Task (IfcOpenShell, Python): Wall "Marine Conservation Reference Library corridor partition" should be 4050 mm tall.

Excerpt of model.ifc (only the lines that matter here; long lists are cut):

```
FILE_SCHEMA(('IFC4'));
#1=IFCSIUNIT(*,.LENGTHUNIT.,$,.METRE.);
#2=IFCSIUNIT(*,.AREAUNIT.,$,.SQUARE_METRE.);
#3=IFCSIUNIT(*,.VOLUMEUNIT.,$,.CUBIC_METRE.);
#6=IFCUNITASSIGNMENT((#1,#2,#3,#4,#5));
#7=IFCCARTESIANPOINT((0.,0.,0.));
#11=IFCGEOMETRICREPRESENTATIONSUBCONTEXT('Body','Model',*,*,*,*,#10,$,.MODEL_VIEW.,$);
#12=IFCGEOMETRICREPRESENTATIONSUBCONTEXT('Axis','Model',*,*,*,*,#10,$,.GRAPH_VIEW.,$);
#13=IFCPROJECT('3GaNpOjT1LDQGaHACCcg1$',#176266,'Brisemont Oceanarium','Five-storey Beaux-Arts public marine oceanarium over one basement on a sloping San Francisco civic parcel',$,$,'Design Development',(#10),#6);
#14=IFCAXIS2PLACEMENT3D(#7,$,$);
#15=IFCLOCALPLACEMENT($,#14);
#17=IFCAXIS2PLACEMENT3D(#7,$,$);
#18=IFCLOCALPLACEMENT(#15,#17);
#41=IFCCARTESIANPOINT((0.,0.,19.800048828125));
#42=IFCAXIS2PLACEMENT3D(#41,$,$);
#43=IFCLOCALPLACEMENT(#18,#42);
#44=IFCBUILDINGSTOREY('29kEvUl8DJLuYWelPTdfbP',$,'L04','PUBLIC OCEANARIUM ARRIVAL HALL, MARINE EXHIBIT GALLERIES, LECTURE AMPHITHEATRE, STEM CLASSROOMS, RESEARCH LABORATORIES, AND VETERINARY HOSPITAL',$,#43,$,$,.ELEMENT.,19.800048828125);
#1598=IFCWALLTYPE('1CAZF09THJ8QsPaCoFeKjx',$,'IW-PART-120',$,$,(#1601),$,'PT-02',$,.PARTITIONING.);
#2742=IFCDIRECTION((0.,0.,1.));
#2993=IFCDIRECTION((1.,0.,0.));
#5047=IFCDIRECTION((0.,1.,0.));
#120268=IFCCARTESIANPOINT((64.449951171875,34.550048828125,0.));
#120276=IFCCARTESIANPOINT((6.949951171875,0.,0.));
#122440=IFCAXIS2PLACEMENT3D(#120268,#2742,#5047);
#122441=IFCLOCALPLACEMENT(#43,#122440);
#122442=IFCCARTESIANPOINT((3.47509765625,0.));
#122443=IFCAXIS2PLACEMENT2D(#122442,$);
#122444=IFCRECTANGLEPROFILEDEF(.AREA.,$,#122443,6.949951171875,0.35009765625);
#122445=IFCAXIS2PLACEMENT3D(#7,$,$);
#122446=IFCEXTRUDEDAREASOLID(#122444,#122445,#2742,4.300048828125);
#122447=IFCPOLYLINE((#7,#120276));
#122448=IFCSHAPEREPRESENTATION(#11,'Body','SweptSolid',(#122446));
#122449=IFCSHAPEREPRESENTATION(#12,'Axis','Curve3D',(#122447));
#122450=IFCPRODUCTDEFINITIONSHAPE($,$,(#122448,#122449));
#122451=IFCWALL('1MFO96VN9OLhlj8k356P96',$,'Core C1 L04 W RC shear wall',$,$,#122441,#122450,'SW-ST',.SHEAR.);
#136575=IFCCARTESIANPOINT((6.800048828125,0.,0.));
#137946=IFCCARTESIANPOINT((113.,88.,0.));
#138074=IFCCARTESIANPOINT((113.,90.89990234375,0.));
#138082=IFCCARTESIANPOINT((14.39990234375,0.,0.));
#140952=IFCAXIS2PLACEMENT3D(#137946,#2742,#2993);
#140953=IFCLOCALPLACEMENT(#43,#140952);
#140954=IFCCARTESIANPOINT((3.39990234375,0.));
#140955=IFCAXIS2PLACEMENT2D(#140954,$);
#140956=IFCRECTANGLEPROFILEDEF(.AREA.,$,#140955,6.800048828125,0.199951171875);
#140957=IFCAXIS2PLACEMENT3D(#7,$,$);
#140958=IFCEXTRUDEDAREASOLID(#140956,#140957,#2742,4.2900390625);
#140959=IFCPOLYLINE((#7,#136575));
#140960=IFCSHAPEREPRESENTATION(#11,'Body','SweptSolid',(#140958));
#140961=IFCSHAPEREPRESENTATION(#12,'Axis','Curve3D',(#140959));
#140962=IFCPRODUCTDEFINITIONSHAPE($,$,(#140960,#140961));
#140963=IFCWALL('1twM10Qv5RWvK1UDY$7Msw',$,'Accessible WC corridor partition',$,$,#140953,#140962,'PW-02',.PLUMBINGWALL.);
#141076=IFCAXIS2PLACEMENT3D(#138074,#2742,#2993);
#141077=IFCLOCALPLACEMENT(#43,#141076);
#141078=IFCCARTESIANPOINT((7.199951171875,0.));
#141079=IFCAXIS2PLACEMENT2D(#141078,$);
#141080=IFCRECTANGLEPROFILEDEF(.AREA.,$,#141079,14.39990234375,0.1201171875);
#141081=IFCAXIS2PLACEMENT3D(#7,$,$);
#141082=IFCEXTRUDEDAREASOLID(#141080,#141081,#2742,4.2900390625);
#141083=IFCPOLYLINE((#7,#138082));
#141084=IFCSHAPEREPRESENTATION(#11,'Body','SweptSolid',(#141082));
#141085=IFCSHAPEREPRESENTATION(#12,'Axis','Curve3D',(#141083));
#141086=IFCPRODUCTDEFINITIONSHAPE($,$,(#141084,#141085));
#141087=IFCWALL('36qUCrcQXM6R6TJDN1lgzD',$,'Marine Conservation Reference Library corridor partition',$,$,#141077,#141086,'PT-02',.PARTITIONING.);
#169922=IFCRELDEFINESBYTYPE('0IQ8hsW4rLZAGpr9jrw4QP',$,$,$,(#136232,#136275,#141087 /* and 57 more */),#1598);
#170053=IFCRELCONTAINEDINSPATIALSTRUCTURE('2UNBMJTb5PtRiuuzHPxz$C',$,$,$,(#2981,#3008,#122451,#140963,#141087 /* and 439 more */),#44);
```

```python
import ifcopenshell
import ifcopenshell.geom
import ifcopenshell.util.representation
import ifcopenshell.util.shape

model = ifcopenshell.open("model.ifc")
settings = ifcopenshell.geom.settings()


def volume(element):
    """Net volume in cubic metres, openings subtracted."""
    shape = ifcopenshell.geom.create_shape(settings, element)
    return ifcopenshell.util.shape.get_volume(shape.geometry)


wall = model.by_guid("36qUCrcQXM6R6TJDN1lgzD")
before = volume(wall)

body = ifcopenshell.util.representation.get_representation(wall, "Model", "Body")
solid = body.Items[0]
old_height = solid.Depth
solid.Depth = 4.05
after = volume(wall)

print(f"height {old_height:g} -> {solid.Depth:g}, volume {before:.3f} -> {after:.3f} m3")

model.write("model_edited.ifc")
```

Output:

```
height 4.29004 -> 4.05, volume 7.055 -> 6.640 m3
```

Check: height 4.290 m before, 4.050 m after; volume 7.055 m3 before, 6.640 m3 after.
